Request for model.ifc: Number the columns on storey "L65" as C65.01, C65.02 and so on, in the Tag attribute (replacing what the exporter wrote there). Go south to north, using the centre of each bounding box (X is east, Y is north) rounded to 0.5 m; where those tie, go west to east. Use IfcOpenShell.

First a look at what the model holds.

```python
import ifcopenshell
import ifcopenshell.util.element
import ifcopenshell.util.placement

model = ifcopenshell.open("model.ifc")
print(model.schema)
storey = next(s for s in model.by_type("IfcBuildingStorey") if s.Name == "L65")
columns = [e for e in ifcopenshell.util.element.get_decomposition(storey) if e.is_a("IfcColumn")]
for e in sorted(columns, key=lambda e: e.id()):
    origin = ifcopenshell.util.placement.get_local_placement(e.ObjectPlacement)[:3, 3]
    print(e.id(), e.Tag, e.Name, origin.round(2) + 0.0, sep=" | ")
```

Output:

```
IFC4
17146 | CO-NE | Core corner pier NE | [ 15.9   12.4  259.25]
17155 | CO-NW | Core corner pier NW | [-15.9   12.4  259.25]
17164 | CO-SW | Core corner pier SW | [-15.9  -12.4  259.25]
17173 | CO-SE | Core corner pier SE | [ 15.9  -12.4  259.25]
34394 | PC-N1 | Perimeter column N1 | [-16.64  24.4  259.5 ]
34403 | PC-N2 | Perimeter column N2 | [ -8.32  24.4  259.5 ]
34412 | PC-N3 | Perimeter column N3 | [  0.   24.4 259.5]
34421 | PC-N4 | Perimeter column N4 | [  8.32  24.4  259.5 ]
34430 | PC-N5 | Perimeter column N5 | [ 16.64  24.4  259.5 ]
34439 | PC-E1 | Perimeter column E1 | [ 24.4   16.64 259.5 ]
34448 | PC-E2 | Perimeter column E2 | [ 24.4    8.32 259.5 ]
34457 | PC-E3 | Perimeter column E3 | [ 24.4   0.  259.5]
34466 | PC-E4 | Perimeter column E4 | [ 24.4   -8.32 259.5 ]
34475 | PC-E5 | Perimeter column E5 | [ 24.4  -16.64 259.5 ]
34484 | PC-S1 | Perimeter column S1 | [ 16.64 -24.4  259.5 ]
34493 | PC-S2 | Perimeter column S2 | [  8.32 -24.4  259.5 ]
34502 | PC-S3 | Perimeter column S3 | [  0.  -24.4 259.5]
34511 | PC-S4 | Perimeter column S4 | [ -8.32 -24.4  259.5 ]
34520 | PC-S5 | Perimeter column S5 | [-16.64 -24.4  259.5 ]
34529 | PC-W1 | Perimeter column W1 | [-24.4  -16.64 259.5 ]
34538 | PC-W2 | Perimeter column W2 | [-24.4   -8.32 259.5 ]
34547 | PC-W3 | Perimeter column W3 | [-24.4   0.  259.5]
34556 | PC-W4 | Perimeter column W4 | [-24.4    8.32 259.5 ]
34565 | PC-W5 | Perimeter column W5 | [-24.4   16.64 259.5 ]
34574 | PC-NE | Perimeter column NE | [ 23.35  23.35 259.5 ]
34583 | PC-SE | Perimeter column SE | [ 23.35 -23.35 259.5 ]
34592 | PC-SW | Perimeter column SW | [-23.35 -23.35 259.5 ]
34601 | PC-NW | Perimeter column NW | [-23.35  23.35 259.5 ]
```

```python
import ifcopenshell
import ifcopenshell.geom
import ifcopenshell.util.element
import ifcopenshell.util.shape

model = ifcopenshell.open("model.ifc")
settings = ifcopenshell.geom.settings()
settings.set("use-world-coords", True)


def centre(element):
    shape = ifcopenshell.geom.create_shape(settings, element)
    return ifcopenshell.util.shape.get_bbox_centroid(shape.geometry)


storey = next(s for s in model.by_type("IfcBuildingStorey") if s.Name == "L65")
columns = [e for e in ifcopenshell.util.element.get_decomposition(storey) if e.is_a("IfcColumn")]

# Insertion points can sit at a corner or the storey origin, so sort by the geometry (in metres).
centres = {e: centre(e) for e in columns}
columns.sort(key=lambda e: (round(centres[e][1] / 0.5), centres[e][0]))

for i, e in enumerate(columns, start=1):
    number = f"C65.{i:02d}"
    e.Tag = number
    print(e.id(), number)

model.write("model_rev.ifc")
```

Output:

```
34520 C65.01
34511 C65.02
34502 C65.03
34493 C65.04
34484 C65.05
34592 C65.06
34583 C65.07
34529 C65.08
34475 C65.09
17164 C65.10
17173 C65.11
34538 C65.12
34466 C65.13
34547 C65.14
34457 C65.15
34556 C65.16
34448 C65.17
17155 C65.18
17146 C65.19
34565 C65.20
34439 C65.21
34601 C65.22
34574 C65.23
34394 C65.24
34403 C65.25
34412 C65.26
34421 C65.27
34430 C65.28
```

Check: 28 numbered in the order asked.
